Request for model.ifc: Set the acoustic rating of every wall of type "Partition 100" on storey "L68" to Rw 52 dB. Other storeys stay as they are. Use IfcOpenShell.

First a look at what the model holds.

```python
import ifcopenshell
import ifcopenshell.util.element

model = ifcopenshell.open("model.ifc")
print(model.schema)
storey = next(s for s in model.by_type("IfcBuildingStorey") if s.Name == "L68")
walls = [e for e in ifcopenshell.util.element.get_decomposition(storey) if e.is_a("IfcWall")]
seen = {}
for e in walls:
    element_type = ifcopenshell.util.element.get_type(e)
    key = (element_type.Name if element_type != e and element_type else None, ifcopenshell.util.element.get_pset(e, "Pset_WallCommon", "AcousticRating"))
    seen[key] = seen.get(key, 0) + 1
for (name, value), count in sorted(seen.items(), key=str):
    print(count, "x", name, "|", value)
```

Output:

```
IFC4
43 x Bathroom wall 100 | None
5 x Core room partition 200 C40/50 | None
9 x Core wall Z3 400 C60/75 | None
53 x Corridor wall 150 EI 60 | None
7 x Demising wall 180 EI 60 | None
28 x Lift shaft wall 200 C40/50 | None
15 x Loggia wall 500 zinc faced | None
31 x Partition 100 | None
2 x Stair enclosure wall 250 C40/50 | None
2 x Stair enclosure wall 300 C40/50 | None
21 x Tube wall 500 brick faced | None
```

```python
import ifcopenshell
import ifcopenshell.api.pset
import ifcopenshell.util.element

model = ifcopenshell.open("model.ifc")

storey = next(s for s in model.by_type("IfcBuildingStorey") if s.Name == "L68")
walls = [e for e in ifcopenshell.util.element.get_decomposition(storey) if e.is_a("IfcWall")]

count = 0
for e in walls:
    element_type = ifcopenshell.util.element.get_type(e)
    if element_type in (None, e) or element_type.Name != "Partition 100":
        continue
    found = ifcopenshell.util.element.get_pset(e, "Pset_WallCommon", should_inherit=False)
    if found:
        pset = model.by_id(found["id"])
        if len(ifcopenshell.util.element.get_elements_by_pset(pset)) > 1:
            pset = ifcopenshell.api.pset.unshare_pset(model, products=[e], pset=pset)[0]
    else:
        pset = ifcopenshell.api.pset.add_pset(model, product=e, name="Pset_WallCommon")
    ifcopenshell.api.pset.edit_pset(model, pset=pset, properties={"AcousticRating": "Rw 52 dB"})
    count += 1

print(count, "walls updated")

model.write("model-out.ifc")
```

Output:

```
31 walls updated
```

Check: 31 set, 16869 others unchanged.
